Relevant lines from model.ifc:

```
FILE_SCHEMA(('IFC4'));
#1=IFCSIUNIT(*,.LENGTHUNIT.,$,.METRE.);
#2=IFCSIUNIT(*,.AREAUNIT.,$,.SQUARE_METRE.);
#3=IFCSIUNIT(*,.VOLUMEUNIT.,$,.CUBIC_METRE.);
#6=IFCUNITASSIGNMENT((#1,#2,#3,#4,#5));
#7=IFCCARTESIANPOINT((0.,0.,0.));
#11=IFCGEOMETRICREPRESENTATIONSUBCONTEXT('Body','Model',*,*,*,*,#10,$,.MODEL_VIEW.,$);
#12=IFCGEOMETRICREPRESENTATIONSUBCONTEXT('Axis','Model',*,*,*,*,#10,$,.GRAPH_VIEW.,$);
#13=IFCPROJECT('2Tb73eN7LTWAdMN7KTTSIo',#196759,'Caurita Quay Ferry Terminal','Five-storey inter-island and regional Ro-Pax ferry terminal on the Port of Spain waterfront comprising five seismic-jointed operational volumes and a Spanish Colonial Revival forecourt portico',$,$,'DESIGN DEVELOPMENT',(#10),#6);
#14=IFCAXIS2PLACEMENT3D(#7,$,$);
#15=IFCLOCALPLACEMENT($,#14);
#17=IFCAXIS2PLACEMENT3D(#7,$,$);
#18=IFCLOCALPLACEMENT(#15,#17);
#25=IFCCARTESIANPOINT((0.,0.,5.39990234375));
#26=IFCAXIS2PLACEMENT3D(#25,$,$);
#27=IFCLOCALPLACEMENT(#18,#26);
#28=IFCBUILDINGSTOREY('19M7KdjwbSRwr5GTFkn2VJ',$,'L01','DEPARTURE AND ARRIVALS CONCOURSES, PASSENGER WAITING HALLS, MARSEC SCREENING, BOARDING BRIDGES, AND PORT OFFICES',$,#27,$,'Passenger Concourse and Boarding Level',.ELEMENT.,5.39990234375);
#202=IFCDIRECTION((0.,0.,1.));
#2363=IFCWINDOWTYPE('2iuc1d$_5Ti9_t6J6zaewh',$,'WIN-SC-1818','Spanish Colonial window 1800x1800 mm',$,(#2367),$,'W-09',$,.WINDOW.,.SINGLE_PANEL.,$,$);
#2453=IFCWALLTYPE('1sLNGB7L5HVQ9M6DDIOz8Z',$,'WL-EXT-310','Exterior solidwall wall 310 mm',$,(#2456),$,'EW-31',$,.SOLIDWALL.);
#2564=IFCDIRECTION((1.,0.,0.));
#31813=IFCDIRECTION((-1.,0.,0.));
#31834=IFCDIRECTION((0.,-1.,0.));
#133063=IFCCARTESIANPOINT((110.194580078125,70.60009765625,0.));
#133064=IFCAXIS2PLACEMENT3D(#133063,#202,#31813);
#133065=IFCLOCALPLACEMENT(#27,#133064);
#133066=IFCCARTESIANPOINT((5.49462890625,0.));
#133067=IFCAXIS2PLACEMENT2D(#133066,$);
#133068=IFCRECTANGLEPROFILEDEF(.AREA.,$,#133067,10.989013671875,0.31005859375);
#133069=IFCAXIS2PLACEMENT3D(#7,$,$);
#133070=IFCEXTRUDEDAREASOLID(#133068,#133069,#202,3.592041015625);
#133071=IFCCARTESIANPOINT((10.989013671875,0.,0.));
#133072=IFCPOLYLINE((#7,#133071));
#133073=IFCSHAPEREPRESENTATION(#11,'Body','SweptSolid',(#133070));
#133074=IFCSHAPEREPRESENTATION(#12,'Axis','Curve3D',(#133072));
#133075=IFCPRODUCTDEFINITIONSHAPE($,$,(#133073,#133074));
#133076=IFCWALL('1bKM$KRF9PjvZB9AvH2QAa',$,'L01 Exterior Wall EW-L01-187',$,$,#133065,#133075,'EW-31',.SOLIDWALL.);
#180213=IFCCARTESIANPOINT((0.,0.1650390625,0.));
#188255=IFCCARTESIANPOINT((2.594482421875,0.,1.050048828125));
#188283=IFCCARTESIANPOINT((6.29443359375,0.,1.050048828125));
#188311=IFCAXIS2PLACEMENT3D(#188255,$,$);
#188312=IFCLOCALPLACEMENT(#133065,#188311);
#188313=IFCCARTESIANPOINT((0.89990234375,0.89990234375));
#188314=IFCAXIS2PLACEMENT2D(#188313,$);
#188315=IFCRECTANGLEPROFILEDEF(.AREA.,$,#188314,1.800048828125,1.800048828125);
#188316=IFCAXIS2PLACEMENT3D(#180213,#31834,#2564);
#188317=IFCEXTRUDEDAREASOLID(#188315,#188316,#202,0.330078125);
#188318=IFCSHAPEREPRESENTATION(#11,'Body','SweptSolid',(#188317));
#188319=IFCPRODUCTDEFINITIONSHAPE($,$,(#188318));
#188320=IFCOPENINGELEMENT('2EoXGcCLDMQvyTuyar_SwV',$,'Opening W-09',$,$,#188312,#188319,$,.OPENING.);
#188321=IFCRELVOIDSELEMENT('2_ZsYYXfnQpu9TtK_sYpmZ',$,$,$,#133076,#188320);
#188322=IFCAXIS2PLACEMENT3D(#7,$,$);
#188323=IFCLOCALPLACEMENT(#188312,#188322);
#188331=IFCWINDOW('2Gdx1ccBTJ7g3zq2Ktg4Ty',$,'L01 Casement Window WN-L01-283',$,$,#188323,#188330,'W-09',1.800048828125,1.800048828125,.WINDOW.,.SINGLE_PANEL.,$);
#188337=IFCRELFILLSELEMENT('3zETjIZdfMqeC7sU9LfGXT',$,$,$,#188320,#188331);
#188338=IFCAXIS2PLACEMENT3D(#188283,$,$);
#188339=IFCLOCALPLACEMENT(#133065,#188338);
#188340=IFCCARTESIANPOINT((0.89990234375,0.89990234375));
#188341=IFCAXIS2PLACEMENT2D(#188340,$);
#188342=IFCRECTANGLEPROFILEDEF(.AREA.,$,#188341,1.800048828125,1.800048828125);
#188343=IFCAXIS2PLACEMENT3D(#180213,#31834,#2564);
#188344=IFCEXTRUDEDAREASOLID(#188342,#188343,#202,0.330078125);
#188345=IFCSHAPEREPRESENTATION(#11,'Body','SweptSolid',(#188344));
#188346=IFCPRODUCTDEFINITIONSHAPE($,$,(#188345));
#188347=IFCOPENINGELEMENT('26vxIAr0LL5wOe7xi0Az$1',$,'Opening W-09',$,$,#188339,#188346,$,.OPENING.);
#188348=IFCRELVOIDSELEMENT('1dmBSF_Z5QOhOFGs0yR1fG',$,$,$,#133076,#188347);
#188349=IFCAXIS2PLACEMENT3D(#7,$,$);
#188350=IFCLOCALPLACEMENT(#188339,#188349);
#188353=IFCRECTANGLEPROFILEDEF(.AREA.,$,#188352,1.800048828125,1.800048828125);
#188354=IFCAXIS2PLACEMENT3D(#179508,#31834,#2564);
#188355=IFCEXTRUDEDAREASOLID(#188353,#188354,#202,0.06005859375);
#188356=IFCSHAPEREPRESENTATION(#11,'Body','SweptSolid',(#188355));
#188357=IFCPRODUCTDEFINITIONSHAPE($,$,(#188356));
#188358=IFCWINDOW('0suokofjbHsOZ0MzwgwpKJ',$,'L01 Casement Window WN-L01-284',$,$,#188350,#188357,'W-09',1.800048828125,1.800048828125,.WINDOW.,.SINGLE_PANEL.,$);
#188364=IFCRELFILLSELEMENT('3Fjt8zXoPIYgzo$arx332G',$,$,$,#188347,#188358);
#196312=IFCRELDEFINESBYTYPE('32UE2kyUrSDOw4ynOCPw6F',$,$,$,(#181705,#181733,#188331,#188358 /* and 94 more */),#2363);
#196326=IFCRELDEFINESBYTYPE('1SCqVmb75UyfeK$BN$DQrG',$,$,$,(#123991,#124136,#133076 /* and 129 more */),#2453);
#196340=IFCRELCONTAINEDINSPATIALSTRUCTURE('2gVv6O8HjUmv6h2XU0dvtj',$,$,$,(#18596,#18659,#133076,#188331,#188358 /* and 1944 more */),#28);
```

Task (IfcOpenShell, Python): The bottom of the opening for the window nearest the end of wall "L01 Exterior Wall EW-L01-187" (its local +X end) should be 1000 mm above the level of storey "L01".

```python
import numpy as np
import ifcopenshell
import ifcopenshell.api.geometry
import ifcopenshell.geom
import ifcopenshell.util.element
import ifcopenshell.util.placement
import ifcopenshell.util.shape
import ifcopenshell.util.unit

model = ifcopenshell.open("model.ifc")
unit_scale = ifcopenshell.util.unit.calculate_unit_scale(model)

window = model.by_guid("0suokofjbHsOZ0MzwgwpKJ")
opening = window.FillsVoids[0].RelatingOpeningElement
storey = ifcopenshell.util.element.get_container(window, ifc_class="IfcBuildingStorey")
level = ifcopenshell.util.placement.get_local_placement(storey.ObjectPlacement)[2, 3]

# The opening's origin need not be at the sill, so measure its lowest point.
shape = ifcopenshell.geom.create_shape(ifcopenshell.geom.settings(), opening)
bottom = ifcopenshell.util.shape.get_shape_bottom_elevation(shape, shape.geometry) / unit_scale
dz = level + 1 / unit_scale - bottom

shift = np.array([0.0, 0.0, dz])
# The window is placed relative to its opening, so it follows when the opening moves.
matrix = ifcopenshell.util.placement.get_local_placement(opening.ObjectPlacement)
matrix[:3, 3] += shift
ifcopenshell.api.geometry.edit_object_placement(
    model, product=opening, matrix=matrix, is_si=False, should_transform_children=True
)

print(f"moved by {dz * unit_scale:+.3f} m")

model.write("model_edited.ifc")
```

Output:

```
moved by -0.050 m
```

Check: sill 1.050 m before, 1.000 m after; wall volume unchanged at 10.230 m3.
